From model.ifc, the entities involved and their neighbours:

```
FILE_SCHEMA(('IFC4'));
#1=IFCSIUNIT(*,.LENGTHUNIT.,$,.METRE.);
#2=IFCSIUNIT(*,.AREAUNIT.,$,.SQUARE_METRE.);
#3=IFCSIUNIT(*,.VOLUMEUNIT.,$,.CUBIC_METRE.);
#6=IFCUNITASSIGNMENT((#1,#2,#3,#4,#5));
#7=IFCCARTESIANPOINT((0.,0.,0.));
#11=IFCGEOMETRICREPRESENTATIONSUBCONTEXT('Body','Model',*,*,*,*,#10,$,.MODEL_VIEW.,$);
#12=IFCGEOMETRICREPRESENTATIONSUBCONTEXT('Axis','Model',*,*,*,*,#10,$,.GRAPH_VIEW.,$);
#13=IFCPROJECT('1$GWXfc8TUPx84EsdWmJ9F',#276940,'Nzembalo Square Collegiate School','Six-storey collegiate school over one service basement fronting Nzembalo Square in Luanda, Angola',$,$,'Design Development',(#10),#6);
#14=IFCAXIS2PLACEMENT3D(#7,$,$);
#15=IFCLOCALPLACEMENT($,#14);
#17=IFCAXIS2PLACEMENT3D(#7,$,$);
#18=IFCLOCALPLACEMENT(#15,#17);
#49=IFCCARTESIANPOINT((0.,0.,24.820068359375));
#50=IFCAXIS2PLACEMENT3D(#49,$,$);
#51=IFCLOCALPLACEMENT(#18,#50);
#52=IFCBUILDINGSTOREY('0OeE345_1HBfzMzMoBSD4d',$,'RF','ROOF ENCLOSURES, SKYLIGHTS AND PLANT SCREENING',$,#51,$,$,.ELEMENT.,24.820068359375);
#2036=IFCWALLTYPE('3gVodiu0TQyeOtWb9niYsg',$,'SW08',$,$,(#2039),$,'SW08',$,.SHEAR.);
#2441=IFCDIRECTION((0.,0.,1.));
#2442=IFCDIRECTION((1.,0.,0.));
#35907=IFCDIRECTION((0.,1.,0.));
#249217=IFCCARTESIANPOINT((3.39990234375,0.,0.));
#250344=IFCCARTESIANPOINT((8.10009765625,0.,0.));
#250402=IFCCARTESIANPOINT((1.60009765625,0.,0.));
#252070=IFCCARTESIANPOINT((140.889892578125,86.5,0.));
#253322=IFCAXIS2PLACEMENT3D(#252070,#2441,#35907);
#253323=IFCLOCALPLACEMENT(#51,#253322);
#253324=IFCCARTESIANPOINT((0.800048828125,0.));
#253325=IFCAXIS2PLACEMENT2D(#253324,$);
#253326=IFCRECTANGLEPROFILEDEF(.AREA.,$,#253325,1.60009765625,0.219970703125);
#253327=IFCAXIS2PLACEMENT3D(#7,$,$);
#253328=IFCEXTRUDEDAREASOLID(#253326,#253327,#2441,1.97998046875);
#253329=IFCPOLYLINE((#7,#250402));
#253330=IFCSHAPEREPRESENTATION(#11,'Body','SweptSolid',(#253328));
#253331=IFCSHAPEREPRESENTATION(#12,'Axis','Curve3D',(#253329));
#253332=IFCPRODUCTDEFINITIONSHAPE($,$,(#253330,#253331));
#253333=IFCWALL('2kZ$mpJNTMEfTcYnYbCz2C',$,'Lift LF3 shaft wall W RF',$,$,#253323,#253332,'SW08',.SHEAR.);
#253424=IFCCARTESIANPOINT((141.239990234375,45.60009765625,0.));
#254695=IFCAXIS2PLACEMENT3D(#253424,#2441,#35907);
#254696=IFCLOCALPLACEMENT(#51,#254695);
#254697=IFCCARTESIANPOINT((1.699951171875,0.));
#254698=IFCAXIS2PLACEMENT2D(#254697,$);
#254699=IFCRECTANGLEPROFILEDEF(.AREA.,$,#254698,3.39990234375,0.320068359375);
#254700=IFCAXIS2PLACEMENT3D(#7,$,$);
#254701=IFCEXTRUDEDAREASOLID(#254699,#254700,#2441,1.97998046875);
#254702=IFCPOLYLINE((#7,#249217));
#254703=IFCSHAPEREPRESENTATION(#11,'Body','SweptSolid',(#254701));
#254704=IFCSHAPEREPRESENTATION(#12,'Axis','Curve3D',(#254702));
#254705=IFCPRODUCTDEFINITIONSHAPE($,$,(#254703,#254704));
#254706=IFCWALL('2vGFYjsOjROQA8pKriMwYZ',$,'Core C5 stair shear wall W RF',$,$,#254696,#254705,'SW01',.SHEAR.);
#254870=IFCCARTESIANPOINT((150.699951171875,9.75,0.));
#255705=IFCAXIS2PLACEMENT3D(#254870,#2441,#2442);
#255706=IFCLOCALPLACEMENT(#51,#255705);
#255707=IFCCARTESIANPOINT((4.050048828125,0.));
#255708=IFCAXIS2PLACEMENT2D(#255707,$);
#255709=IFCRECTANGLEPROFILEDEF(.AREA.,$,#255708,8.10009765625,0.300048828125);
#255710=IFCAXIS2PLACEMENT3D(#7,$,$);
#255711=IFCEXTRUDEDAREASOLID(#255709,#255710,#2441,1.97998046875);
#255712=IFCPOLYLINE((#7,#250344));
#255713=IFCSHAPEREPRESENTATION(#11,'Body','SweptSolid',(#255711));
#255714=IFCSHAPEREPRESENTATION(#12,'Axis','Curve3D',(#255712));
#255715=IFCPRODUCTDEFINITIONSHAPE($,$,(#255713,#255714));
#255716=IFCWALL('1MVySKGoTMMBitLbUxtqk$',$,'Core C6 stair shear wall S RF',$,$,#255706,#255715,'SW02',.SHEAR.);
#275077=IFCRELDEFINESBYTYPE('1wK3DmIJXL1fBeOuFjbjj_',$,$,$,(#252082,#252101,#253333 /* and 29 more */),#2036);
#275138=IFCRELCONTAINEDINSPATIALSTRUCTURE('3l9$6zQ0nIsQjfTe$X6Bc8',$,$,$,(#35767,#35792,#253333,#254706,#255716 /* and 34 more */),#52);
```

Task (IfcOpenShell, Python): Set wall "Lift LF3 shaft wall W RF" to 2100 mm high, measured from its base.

```python
import ifcopenshell
import ifcopenshell.geom
import ifcopenshell.util.representation
import ifcopenshell.util.shape

model = ifcopenshell.open("model.ifc")
settings = ifcopenshell.geom.settings()


def volume(element):
    """Net volume in cubic metres, openings subtracted."""
    shape = ifcopenshell.geom.create_shape(settings, element)
    return ifcopenshell.util.shape.get_volume(shape.geometry)


wall = model.by_guid("2kZ$mpJNTMEfTcYnYbCz2C")
before = volume(wall)

body = ifcopenshell.util.representation.get_representation(wall, "Model", "Body")
solid = body.Items[0]
old_height = solid.Depth
solid.Depth = 2.1
after = volume(wall)

print(f"height {old_height:g} -> {solid.Depth:g}, volume {before:.3f} -> {after:.3f} m3")

model.write("model_edited.ifc")
```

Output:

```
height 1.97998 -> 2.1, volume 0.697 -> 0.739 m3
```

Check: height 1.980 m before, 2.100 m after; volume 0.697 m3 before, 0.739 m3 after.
